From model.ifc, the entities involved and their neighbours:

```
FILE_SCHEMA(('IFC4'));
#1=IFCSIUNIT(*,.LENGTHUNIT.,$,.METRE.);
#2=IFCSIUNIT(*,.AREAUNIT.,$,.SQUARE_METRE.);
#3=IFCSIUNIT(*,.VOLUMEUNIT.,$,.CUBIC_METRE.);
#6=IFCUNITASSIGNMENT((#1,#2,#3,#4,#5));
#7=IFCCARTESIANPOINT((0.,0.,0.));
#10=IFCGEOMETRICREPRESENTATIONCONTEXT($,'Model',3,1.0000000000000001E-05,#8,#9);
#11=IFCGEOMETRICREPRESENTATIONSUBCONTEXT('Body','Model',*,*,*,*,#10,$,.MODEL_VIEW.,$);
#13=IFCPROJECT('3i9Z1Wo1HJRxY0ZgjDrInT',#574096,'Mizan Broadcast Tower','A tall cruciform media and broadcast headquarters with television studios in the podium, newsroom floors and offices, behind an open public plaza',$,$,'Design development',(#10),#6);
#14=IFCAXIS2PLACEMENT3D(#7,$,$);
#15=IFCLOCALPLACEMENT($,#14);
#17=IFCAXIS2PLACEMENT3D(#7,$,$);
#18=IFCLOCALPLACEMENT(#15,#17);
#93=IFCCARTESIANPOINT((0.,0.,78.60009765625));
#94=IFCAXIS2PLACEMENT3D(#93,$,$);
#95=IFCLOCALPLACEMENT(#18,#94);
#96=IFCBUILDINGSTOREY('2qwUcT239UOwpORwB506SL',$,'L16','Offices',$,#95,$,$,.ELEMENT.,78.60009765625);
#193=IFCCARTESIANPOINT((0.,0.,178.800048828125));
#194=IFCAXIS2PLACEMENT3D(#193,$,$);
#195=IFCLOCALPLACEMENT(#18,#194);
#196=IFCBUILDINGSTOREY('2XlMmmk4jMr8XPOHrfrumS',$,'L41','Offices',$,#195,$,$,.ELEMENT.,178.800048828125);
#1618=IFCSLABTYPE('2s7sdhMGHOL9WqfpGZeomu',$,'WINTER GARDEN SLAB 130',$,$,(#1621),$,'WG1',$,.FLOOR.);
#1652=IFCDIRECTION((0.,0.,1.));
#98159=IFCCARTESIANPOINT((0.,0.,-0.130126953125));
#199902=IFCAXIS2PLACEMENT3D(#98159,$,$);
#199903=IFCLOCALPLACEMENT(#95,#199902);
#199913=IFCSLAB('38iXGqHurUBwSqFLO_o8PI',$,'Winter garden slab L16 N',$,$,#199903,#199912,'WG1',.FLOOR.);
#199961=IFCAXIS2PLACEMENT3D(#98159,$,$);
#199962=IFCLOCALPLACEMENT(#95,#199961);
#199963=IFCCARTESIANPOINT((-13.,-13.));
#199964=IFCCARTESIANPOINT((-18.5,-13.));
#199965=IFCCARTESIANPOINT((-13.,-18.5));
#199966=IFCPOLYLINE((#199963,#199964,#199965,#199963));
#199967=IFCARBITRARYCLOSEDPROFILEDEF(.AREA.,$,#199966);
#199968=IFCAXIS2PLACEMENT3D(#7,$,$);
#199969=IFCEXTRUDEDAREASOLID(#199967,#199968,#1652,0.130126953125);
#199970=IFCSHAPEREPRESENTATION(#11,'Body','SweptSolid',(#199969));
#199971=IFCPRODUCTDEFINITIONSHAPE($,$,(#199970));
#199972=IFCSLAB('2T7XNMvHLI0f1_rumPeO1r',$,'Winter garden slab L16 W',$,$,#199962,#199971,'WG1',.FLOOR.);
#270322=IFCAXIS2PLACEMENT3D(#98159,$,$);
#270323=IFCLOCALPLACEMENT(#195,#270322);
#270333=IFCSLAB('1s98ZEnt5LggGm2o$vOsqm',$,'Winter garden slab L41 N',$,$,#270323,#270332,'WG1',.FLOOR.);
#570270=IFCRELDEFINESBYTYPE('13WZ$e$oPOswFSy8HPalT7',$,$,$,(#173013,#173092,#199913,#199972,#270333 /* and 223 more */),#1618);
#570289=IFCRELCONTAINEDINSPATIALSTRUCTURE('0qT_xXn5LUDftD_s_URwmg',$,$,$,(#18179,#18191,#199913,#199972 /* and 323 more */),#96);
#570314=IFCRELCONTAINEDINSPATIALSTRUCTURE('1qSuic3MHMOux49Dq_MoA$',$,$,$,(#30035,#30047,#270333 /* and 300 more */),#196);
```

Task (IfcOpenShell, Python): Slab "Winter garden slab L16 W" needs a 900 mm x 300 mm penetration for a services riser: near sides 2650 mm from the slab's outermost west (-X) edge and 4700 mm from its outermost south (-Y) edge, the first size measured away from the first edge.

```python
import numpy as np
import ifcopenshell
import ifcopenshell.api.feature
import ifcopenshell.api.geometry
import ifcopenshell.api.root
import ifcopenshell.geom
import ifcopenshell.util.placement
import ifcopenshell.util.representation
import ifcopenshell.util.shape
import ifcopenshell.util.unit

model = ifcopenshell.open("model.ifc")
unit_scale = ifcopenshell.util.unit.calculate_unit_scale(model)
settings = ifcopenshell.geom.settings()


def volume(element):
    """Net volume in cubic metres, openings subtracted."""
    shape = ifcopenshell.geom.create_shape(settings, element)
    return ifcopenshell.util.shape.get_volume(shape.geometry)


slab = model.by_guid("2T7XNMvHLI0f1_rumPeO1r")
before = volume(slab)

# Extent in the slab's own axes, in metres. The edges named are its -X and -Y sides.
slab_shape = ifcopenshell.geom.create_shape(settings, slab)
vertices = ifcopenshell.util.shape.get_vertices(slab_shape.geometry)
x_min, y_min, bottom = vertices.min(axis=0)
top = vertices[:, 2].max()

opening = ifcopenshell.api.root.create_entity(model, ifc_class="IfcOpeningElement", name="Services riser opening", predefined_type="OPENING")
context = ifcopenshell.util.representation.get_context(model, "Model", "Body", "MODEL_VIEW")
width, depth = 0.9, 0.3
outline = [(0.0, 0.0), (width, 0.0), (width, depth), (0.0, depth), (0.0, 0.0)]
# Overshoot both faces by 50 mm so the cut is clean.
shape = ifcopenshell.api.geometry.add_slab_representation(
    model, context=context, depth=top - bottom + 0.1, polyline=outline
)
ifcopenshell.api.geometry.assign_representation(model, product=opening, representation=shape)

matrix = ifcopenshell.util.placement.get_local_placement(slab.ObjectPlacement)
matrix[:, 3] = matrix @ np.append(np.array([x_min + 2.65, y_min + 4.7, bottom - 0.05]) / unit_scale, 1.0)
ifcopenshell.api.geometry.edit_object_placement(model, product=opening, matrix=matrix, is_si=False)
ifcopenshell.api.feature.add_feature(model, feature=opening, element=slab)

after = volume(slab)

print(f"slab volume {before:.3f} -> {after:.3f} m3")

model.write("model_rev.ifc")
```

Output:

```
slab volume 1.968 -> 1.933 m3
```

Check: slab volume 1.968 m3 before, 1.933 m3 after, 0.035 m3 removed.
